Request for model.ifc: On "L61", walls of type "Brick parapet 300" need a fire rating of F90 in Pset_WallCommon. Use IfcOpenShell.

First a look at what the model holds.

```python
import ifcopenshell
import ifcopenshell.util.element

model = ifcopenshell.open("model.ifc")
print(model.schema)
storey = next(s for s in model.by_type("IfcBuildingStorey") if s.Name == "L61")
walls = [e for e in ifcopenshell.util.element.get_decomposition(storey) if e.is_a("IfcWall")]
seen = {}
for e in walls:
    element_type = ifcopenshell.util.element.get_type(e)
    key = (element_type.Name if element_type != e and element_type else None, ifcopenshell.util.element.get_pset(e, "Pset_WallCommon", "FireRating"))
    seen[key] = seen.get(key, 0) + 1
for (name, value), count in sorted(seen.items(), key=str):
    print(count, "x", name, "|", value)
```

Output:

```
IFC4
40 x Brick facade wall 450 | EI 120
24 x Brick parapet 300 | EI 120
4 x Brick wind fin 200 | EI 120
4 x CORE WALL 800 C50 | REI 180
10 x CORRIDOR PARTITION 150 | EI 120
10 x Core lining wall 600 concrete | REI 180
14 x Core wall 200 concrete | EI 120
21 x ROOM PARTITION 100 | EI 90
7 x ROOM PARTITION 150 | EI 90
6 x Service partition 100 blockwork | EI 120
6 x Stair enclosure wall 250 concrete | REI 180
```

```python
import ifcopenshell
import ifcopenshell.api.pset
import ifcopenshell.util.element

model = ifcopenshell.open("model.ifc")

storey = next(s for s in model.by_type("IfcBuildingStorey") if s.Name == "L61")
walls = [e for e in ifcopenshell.util.element.get_decomposition(storey) if e.is_a("IfcWall")]

count = 0
for e in walls:
    element_type = ifcopenshell.util.element.get_type(e)
    if element_type in (None, e) or element_type.Name != "Brick parapet 300":
        continue
    found = ifcopenshell.util.element.get_pset(e, "Pset_WallCommon", should_inherit=False)
    if found:
        pset = model.by_id(found["id"])
        if len(ifcopenshell.util.element.get_elements_by_pset(pset)) > 1:
            pset = ifcopenshell.api.pset.unshare_pset(model, products=[e], pset=pset)[0]
    else:
        pset = ifcopenshell.api.pset.add_pset(model, product=e, name="Pset_WallCommon")
    ifcopenshell.api.pset.edit_pset(model, pset=pset, properties={"FireRating": "F90"})
    count += 1

print(count, "walls updated")

model.write("model_edited.ifc")
```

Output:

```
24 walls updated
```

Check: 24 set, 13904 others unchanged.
